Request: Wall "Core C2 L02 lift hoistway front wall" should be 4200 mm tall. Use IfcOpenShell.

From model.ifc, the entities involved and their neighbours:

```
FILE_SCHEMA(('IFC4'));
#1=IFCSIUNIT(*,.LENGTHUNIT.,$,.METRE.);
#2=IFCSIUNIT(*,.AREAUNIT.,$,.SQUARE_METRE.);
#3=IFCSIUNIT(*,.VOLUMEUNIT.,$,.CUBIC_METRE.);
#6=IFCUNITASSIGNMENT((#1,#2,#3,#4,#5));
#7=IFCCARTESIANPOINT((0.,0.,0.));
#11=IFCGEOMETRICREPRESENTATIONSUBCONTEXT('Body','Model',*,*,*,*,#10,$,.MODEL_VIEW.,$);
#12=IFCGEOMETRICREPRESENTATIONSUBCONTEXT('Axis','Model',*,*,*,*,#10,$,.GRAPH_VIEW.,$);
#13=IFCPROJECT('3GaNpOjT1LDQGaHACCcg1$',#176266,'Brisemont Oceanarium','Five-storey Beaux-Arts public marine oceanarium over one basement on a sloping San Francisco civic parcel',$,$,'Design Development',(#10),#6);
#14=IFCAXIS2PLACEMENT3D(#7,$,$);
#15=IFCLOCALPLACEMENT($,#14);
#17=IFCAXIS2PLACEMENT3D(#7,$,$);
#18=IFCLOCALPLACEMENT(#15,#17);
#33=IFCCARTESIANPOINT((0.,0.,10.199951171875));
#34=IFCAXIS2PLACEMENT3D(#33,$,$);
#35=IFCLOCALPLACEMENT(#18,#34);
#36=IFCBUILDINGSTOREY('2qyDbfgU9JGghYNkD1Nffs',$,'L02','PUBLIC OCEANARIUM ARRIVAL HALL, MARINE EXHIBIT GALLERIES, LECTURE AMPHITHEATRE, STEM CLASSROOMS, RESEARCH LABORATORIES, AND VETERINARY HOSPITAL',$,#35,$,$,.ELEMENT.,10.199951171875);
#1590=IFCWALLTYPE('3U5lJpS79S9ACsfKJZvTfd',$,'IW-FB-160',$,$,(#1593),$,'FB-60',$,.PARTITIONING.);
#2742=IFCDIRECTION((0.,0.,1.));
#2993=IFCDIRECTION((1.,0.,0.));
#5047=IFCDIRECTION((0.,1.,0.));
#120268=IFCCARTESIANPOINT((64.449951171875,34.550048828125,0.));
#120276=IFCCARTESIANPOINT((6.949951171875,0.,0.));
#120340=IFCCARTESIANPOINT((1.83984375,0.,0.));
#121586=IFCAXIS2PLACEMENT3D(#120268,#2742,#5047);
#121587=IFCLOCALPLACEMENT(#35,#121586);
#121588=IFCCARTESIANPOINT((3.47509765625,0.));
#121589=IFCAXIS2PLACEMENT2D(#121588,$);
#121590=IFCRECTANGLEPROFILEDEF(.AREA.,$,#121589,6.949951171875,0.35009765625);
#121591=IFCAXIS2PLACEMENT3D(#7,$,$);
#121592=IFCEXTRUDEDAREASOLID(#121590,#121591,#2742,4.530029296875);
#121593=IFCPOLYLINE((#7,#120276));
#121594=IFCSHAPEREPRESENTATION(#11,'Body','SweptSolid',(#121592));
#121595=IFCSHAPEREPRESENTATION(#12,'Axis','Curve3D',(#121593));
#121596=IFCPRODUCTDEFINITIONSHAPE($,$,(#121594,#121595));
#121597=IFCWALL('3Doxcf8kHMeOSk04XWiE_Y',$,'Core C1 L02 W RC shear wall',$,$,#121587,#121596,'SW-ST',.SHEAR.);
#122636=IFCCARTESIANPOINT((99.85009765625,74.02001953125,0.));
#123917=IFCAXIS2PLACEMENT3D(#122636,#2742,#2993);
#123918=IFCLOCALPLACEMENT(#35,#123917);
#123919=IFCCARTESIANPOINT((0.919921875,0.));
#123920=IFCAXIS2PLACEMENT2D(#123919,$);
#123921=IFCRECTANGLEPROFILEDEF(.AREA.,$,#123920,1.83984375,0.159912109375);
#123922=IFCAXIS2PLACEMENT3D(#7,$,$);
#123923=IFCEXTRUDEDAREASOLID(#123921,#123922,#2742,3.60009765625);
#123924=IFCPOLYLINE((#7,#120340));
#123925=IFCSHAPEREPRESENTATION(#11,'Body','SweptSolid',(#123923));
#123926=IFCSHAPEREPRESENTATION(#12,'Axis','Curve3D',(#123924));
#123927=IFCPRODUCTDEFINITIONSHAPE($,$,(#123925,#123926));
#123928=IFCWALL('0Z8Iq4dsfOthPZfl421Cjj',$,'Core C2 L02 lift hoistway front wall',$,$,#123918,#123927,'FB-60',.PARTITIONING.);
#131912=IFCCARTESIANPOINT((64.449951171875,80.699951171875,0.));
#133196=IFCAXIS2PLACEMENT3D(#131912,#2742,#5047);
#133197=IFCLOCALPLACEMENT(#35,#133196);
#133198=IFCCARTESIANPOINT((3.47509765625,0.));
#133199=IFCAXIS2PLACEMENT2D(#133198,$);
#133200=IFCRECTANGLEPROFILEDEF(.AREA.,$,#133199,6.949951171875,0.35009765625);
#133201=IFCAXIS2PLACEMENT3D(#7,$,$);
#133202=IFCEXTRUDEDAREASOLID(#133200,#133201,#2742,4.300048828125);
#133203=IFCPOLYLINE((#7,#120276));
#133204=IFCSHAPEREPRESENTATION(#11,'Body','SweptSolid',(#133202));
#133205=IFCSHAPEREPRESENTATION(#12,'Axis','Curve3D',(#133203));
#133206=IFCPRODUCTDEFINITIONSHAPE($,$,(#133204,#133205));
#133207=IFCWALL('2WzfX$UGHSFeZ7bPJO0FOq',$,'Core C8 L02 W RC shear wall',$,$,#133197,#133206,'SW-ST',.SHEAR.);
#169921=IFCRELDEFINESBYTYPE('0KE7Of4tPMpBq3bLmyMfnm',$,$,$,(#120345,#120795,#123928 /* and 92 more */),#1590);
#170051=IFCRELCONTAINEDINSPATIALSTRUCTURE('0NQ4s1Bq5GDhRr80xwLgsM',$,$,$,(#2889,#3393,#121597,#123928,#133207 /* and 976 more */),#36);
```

```python
import ifcopenshell
import ifcopenshell.geom
import ifcopenshell.util.representation
import ifcopenshell.util.shape
import ifcopenshell.util.unit

model = ifcopenshell.open("model.ifc")
unit_scale = ifcopenshell.util.unit.calculate_unit_scale(model)
settings = ifcopenshell.geom.settings()


def volume(element):
    """Net volume in cubic metres, openings subtracted."""
    shape = ifcopenshell.geom.create_shape(settings, element)
    return ifcopenshell.util.shape.get_volume(shape.geometry)


wall = model.by_guid("0Z8Iq4dsfOthPZfl421Cjj")
before = volume(wall)

body = ifcopenshell.util.representation.get_representation(wall, "Model", "Body")
solid = body.Items[0]
old_height = solid.Depth
solid.Depth = 4.2 / unit_scale
after = volume(wall)

print(f"height {old_height:g} -> {solid.Depth:g}, volume {before:.3f} -> {after:.3f} m3")

model.write("model_rev.ifc")
```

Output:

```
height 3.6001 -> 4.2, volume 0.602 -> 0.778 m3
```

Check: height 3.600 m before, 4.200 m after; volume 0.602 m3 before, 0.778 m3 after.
